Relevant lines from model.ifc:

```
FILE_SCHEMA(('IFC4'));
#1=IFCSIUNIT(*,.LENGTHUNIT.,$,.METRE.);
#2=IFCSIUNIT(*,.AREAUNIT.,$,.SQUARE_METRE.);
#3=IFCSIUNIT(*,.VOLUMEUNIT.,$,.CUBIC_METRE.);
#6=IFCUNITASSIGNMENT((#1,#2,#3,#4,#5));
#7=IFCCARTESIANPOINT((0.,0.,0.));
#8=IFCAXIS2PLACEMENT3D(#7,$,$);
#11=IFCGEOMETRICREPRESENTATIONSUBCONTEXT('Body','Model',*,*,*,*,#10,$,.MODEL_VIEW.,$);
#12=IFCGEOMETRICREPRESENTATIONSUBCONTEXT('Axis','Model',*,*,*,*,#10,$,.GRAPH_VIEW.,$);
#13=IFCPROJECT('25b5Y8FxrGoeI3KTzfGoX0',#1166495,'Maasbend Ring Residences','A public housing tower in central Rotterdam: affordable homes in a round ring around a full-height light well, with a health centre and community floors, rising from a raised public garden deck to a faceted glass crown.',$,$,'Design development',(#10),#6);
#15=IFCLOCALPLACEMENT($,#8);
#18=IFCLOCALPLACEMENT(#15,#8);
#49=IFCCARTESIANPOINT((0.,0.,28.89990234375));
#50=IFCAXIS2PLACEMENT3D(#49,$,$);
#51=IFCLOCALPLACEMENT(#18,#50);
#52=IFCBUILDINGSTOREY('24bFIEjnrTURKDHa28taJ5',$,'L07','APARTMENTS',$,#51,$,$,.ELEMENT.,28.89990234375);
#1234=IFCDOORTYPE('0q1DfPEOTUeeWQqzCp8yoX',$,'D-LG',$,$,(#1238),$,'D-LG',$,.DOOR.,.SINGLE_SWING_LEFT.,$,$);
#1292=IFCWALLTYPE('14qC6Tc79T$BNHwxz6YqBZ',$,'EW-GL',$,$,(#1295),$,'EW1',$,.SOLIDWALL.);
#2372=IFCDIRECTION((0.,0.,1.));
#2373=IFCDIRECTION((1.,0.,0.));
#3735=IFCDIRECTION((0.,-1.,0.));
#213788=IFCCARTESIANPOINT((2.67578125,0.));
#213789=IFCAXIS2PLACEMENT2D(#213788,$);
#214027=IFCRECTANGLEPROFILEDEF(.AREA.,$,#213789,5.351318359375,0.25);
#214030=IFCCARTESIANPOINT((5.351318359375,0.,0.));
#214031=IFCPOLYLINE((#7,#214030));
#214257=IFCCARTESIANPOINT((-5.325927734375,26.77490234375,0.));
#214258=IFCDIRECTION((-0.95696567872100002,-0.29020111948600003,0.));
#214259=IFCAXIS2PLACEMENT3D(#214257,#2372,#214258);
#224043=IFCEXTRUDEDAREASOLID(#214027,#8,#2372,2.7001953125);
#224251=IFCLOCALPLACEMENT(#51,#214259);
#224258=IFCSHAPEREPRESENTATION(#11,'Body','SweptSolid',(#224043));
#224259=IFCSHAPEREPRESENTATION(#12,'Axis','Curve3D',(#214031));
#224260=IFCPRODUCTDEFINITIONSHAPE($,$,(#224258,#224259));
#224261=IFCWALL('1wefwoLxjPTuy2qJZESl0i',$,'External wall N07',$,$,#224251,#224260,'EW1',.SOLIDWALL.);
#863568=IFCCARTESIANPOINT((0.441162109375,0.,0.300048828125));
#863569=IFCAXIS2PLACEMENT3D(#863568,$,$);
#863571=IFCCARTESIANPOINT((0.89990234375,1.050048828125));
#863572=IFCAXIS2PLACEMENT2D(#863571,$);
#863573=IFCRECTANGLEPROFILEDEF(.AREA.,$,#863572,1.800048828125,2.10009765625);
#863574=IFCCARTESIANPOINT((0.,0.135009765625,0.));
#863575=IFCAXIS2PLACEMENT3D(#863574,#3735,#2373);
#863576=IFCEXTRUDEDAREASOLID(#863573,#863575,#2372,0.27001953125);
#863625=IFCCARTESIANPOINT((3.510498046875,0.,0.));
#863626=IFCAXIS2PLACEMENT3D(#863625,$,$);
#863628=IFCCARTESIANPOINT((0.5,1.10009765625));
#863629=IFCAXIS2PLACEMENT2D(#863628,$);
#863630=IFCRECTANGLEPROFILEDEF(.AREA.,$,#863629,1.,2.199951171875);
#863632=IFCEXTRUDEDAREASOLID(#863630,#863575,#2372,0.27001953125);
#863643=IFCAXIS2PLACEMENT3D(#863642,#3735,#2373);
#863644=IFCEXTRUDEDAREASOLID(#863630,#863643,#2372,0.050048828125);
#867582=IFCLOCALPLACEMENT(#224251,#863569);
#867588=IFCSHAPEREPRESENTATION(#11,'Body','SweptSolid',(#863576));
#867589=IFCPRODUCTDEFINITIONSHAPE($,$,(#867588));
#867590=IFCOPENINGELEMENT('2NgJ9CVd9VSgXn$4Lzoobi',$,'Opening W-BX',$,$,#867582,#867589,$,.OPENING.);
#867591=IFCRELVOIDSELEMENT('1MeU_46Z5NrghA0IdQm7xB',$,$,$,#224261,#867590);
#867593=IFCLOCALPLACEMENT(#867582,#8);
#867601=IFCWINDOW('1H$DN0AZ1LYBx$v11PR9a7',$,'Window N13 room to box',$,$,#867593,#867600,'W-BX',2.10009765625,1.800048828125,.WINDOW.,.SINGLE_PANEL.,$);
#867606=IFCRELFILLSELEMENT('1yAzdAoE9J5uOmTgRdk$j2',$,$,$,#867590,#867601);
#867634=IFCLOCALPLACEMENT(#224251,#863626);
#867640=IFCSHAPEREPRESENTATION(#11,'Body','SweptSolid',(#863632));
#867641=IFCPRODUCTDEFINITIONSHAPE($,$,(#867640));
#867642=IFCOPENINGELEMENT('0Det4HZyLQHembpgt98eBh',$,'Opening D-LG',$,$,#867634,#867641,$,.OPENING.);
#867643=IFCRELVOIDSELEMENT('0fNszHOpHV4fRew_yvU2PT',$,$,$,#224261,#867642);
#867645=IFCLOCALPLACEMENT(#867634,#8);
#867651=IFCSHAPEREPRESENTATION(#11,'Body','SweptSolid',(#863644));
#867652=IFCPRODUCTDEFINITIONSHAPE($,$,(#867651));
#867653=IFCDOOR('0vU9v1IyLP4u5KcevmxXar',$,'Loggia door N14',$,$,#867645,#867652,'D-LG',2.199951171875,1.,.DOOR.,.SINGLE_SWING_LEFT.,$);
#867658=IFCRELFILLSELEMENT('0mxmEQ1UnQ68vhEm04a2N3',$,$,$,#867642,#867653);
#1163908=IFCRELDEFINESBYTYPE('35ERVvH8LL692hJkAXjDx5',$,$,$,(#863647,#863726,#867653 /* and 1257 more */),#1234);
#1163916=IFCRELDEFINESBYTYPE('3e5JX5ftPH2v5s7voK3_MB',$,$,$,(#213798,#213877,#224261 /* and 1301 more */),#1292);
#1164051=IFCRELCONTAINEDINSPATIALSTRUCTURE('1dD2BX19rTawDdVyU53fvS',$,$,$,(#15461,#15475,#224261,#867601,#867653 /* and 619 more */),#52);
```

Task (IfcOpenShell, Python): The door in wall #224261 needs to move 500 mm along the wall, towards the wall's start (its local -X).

```python
import ifcopenshell
import ifcopenshell.api.geometry
import ifcopenshell.util.placement
import ifcopenshell.util.unit

model = ifcopenshell.open("model.ifc")
unit_scale = ifcopenshell.util.unit.calculate_unit_scale(model)

door = model.by_id(867653)
opening = door.FillsVoids[0].RelatingOpeningElement
wall = opening.VoidsElements[0].RelatingBuildingElement

wall_matrix = ifcopenshell.util.placement.get_local_placement(wall.ObjectPlacement)
shift = wall_matrix[:3, 0] * -0.5 / unit_scale
before = ifcopenshell.util.placement.get_local_placement(door.ObjectPlacement)[:3, 3].copy()

# The door is placed relative to its opening, so it follows when the opening moves.
matrix = ifcopenshell.util.placement.get_local_placement(opening.ObjectPlacement)
matrix[:3, 3] += shift
ifcopenshell.api.geometry.edit_object_placement(
    model, product=opening, matrix=matrix, is_si=False, should_transform_children=True
)

after = ifcopenshell.util.placement.get_local_placement(door.ObjectPlacement)[:3, 3]
print("door moved by", (after - before).round(3) + 0.0)

model.write("model_rev.ifc")
```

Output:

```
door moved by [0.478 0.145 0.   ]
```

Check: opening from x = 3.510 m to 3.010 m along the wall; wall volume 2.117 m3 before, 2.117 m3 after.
